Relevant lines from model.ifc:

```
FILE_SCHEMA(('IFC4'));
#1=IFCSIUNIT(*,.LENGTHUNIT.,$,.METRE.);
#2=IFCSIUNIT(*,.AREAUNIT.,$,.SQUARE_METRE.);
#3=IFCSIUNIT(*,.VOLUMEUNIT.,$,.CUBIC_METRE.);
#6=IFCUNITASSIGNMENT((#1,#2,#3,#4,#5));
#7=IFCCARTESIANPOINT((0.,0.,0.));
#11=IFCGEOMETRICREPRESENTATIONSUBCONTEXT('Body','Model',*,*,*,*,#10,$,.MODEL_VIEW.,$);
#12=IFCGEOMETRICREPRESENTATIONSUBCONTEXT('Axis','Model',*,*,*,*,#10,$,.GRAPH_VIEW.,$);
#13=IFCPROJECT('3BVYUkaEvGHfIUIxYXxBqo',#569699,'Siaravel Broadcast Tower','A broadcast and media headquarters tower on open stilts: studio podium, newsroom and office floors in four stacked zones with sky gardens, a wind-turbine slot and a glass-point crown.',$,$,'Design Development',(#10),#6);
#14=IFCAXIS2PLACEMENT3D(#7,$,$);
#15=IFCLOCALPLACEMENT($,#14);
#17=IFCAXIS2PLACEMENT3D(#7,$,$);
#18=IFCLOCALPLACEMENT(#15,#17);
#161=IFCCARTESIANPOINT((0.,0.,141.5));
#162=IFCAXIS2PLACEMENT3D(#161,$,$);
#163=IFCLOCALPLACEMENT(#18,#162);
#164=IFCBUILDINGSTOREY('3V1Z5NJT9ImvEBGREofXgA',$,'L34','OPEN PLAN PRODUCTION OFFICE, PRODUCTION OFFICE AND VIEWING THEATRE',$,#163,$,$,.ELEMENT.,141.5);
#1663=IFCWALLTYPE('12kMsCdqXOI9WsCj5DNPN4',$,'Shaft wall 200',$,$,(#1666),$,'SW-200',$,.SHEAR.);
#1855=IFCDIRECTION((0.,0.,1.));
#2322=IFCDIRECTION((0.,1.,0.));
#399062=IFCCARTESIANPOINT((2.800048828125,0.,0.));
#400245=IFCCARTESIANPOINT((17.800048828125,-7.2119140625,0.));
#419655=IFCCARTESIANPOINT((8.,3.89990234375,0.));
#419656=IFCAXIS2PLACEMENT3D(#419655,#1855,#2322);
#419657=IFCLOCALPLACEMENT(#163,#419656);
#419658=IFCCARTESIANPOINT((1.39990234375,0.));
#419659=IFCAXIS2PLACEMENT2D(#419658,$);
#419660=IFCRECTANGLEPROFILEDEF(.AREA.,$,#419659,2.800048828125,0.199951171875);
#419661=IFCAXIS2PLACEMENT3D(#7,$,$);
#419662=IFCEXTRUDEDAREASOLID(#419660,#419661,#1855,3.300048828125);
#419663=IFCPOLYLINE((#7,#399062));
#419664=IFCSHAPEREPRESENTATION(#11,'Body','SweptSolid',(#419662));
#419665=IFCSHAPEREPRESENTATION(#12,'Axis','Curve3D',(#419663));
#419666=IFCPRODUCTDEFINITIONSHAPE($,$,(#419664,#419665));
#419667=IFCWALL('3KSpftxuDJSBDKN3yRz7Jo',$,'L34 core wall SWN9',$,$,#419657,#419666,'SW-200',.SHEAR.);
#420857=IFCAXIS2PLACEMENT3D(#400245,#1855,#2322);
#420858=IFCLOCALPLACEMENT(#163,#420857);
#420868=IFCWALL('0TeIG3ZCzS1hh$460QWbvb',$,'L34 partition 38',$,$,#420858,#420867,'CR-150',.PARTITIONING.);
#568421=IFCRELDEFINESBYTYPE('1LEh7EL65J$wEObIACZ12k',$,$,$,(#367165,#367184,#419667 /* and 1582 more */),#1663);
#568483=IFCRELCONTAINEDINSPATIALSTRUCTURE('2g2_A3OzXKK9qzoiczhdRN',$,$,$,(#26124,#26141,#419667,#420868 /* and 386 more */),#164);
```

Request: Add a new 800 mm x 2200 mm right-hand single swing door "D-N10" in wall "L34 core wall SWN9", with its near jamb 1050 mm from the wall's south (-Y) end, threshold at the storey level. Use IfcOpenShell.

```python
import numpy as np
import ifcopenshell
import ifcopenshell.api.feature
import ifcopenshell.api.geometry
import ifcopenshell.api.root
import ifcopenshell.api.spatial
import ifcopenshell.geom
import ifcopenshell.util.element
import ifcopenshell.util.placement
import ifcopenshell.util.representation
import ifcopenshell.util.shape
import ifcopenshell.util.unit

model = ifcopenshell.open("model.ifc")
unit_scale = ifcopenshell.util.unit.calculate_unit_scale(model)
settings = ifcopenshell.geom.settings()


def volume(element):
    """Net volume in cubic metres, openings subtracted."""
    shape = ifcopenshell.geom.create_shape(settings, element)
    return ifcopenshell.util.shape.get_volume(shape.geometry)


wall = model.by_guid("3KSpftxuDJSBDKN3yRz7Jo")
storey = ifcopenshell.util.element.get_container(wall, ifc_class="IfcBuildingStorey")
context = ifcopenshell.util.representation.get_context(model, "Model", "Body", "MODEL_VIEW")
before = volume(wall)

width, height, from_end, sill = 0.8, 2.2, 1.05, 0.0  # metres

# The wall runs along its own X axis, and the end named is its -X end.
wall_shape = ifcopenshell.geom.create_shape(settings, wall)
x, y, z = ifcopenshell.util.shape.get_vertices(wall_shape.geometry).T
start = x.min() + from_end
face, thickness = float(y.min()), float(y.max() - y.min())
wall_matrix = ifcopenshell.util.placement.get_local_placement(wall.ObjectPlacement)
level = ifcopenshell.util.placement.get_local_placement(storey.ObjectPlacement)[2, 3]


def in_wall(x, y):
    """Placement at x, y metres in the wall's axes, at sill height."""
    matrix = wall_matrix.copy()
    matrix[:, 3] = wall_matrix @ np.array([x / unit_scale, y / unit_scale, 0.0, 1.0])
    matrix[2, 3] = level + sill / unit_scale
    return matrix


# Opening: a box that overshoots both wall faces by 50 mm.
opening = ifcopenshell.api.root.create_entity(model, ifc_class="IfcOpeningElement", predefined_type="OPENING")
box = ifcopenshell.api.geometry.add_wall_representation(
    model, context=context, length=width, height=height, thickness=thickness + 0.1
)
ifcopenshell.api.geometry.assign_representation(model, product=opening, representation=box)
ifcopenshell.api.geometry.edit_object_placement(model, product=opening, matrix=in_wall(start, face - 0.05), is_si=False)
ifcopenshell.api.feature.add_feature(model, feature=opening, element=wall)

door = ifcopenshell.api.root.create_entity(model, ifc_class="IfcDoor", name="D-N10", predefined_type="DOOR")
door.OverallWidth, door.OverallHeight = width / unit_scale, height / unit_scale
door.OperationType = "SINGLE_SWING_RIGHT"
body = ifcopenshell.api.geometry.add_door_representation(
    model,
    context=context,
    overall_width=door.OverallWidth,
    overall_height=door.OverallHeight,
    operation_type="SINGLE_SWING_RIGHT",
    lining_properties={"LiningDepth": thickness / unit_scale, "ThresholdDepth": thickness / unit_scale},
)
ifcopenshell.api.geometry.assign_representation(model, product=door, representation=body)
ifcopenshell.api.spatial.assign_container(model, products=[door], relating_structure=storey)
ifcopenshell.api.feature.add_filling(model, opening=opening, element=door)

# The lining spans the wall, so the door starts at the wall face.
ifcopenshell.api.geometry.edit_object_placement(model, product=door, matrix=in_wall(start, face), is_si=False)

after = volume(wall)

print(f"wall volume {before:.3f} -> {after:.3f} m3")

model.write("model_v2.ifc")
```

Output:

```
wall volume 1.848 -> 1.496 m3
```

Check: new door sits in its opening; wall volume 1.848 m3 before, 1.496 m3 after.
